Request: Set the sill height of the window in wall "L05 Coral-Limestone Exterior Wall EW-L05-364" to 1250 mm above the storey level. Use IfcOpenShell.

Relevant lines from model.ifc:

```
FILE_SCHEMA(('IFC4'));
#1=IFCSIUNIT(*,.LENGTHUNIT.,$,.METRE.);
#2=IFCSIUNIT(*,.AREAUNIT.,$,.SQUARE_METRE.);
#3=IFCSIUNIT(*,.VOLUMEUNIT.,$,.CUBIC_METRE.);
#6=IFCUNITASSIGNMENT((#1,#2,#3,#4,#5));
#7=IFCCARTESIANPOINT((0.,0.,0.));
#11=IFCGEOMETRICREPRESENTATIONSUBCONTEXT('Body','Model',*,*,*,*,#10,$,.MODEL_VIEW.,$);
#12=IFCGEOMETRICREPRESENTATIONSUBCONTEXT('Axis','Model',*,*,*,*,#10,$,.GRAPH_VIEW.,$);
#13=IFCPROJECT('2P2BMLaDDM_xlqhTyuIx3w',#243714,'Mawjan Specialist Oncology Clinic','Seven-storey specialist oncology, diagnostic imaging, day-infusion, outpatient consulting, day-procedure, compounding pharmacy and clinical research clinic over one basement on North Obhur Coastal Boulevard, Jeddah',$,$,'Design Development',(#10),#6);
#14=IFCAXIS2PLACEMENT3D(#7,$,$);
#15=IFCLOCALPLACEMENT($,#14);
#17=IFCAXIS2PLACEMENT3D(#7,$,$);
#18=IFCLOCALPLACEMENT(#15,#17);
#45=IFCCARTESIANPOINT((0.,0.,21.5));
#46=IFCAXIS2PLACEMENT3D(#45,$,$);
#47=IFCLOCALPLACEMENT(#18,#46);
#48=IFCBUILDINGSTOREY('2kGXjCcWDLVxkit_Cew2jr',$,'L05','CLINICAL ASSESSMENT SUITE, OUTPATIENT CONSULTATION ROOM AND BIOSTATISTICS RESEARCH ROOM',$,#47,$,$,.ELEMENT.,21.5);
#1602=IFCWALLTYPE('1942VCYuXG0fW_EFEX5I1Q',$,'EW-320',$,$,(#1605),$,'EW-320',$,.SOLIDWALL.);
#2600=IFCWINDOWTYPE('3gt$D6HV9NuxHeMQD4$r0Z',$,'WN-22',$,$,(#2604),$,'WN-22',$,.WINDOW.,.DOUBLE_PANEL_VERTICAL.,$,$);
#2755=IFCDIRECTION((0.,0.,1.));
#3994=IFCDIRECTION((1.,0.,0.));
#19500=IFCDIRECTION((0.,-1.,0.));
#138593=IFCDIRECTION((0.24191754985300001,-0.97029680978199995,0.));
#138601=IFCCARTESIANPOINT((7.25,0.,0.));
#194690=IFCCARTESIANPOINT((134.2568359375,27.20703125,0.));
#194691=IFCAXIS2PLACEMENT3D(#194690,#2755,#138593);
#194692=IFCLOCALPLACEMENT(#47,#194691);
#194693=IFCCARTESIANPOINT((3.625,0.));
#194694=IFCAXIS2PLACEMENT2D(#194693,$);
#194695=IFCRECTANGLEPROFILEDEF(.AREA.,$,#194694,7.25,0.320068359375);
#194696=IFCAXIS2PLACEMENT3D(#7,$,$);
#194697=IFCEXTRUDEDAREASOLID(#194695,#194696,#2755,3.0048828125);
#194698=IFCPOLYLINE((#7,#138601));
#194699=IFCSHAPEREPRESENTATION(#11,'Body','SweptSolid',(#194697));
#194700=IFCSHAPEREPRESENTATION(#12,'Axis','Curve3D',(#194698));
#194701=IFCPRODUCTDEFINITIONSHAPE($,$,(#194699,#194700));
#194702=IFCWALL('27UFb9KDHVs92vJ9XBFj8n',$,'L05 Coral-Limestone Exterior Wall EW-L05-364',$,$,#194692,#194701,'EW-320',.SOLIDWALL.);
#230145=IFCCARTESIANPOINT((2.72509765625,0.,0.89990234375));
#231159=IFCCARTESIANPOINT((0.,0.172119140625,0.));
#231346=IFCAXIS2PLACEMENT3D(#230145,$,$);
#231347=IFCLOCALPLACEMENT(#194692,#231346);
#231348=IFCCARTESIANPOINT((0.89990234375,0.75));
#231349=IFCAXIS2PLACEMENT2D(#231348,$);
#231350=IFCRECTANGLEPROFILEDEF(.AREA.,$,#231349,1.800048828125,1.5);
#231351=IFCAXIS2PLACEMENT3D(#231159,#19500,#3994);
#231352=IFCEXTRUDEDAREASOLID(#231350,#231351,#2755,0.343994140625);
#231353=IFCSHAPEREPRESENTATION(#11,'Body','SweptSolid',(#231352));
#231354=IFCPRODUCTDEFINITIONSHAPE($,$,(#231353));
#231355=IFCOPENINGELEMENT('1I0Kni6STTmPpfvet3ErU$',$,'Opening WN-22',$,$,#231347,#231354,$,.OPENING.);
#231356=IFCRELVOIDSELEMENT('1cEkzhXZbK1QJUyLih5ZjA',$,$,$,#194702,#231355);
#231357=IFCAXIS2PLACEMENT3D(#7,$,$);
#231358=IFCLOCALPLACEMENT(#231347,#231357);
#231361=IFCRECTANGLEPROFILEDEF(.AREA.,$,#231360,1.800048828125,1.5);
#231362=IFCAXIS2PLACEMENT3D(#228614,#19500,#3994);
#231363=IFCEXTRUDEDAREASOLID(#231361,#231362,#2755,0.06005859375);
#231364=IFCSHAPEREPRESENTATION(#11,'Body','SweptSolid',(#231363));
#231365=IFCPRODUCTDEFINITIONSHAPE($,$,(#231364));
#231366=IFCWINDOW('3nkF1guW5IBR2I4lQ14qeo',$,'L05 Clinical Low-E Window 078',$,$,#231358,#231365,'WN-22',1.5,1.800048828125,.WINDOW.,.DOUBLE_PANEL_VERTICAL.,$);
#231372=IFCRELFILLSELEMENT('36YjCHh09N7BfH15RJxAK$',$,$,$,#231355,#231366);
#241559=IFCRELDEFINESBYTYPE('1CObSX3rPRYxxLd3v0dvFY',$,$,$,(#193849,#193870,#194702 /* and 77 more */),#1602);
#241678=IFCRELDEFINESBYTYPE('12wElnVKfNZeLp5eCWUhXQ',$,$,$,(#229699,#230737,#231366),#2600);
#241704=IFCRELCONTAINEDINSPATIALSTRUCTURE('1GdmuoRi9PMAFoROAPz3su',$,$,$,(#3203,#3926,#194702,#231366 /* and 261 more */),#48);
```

```python
import numpy as np
import ifcopenshell
import ifcopenshell.api.geometry
import ifcopenshell.geom
import ifcopenshell.util.element
import ifcopenshell.util.placement
import ifcopenshell.util.shape
import ifcopenshell.util.unit

model = ifcopenshell.open("model.ifc")
unit_scale = ifcopenshell.util.unit.calculate_unit_scale(model)

window = model.by_guid("3nkF1guW5IBR2I4lQ14qeo")
opening = window.FillsVoids[0].RelatingOpeningElement
storey = ifcopenshell.util.element.get_container(window, ifc_class="IfcBuildingStorey")
level = ifcopenshell.util.placement.get_local_placement(storey.ObjectPlacement)[2, 3]

# The opening's origin need not be at the sill, so measure its lowest point.
shape = ifcopenshell.geom.create_shape(ifcopenshell.geom.settings(), opening)
bottom = ifcopenshell.util.shape.get_shape_bottom_elevation(shape, shape.geometry) / unit_scale
dz = level + 1.25 - bottom

shift = np.array([0.0, 0.0, dz])
# The window is placed relative to its opening, so it follows when the opening moves.
matrix = ifcopenshell.util.placement.get_local_placement(opening.ObjectPlacement)
matrix[:3, 3] += shift
ifcopenshell.api.geometry.edit_object_placement(
    model, product=opening, matrix=matrix, is_si=False, should_transform_children=True
)

print(f"moved by {dz * unit_scale:+.3f} m")

model.write("model_updated.ifc")
```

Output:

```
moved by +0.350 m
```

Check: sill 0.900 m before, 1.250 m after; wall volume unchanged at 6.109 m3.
